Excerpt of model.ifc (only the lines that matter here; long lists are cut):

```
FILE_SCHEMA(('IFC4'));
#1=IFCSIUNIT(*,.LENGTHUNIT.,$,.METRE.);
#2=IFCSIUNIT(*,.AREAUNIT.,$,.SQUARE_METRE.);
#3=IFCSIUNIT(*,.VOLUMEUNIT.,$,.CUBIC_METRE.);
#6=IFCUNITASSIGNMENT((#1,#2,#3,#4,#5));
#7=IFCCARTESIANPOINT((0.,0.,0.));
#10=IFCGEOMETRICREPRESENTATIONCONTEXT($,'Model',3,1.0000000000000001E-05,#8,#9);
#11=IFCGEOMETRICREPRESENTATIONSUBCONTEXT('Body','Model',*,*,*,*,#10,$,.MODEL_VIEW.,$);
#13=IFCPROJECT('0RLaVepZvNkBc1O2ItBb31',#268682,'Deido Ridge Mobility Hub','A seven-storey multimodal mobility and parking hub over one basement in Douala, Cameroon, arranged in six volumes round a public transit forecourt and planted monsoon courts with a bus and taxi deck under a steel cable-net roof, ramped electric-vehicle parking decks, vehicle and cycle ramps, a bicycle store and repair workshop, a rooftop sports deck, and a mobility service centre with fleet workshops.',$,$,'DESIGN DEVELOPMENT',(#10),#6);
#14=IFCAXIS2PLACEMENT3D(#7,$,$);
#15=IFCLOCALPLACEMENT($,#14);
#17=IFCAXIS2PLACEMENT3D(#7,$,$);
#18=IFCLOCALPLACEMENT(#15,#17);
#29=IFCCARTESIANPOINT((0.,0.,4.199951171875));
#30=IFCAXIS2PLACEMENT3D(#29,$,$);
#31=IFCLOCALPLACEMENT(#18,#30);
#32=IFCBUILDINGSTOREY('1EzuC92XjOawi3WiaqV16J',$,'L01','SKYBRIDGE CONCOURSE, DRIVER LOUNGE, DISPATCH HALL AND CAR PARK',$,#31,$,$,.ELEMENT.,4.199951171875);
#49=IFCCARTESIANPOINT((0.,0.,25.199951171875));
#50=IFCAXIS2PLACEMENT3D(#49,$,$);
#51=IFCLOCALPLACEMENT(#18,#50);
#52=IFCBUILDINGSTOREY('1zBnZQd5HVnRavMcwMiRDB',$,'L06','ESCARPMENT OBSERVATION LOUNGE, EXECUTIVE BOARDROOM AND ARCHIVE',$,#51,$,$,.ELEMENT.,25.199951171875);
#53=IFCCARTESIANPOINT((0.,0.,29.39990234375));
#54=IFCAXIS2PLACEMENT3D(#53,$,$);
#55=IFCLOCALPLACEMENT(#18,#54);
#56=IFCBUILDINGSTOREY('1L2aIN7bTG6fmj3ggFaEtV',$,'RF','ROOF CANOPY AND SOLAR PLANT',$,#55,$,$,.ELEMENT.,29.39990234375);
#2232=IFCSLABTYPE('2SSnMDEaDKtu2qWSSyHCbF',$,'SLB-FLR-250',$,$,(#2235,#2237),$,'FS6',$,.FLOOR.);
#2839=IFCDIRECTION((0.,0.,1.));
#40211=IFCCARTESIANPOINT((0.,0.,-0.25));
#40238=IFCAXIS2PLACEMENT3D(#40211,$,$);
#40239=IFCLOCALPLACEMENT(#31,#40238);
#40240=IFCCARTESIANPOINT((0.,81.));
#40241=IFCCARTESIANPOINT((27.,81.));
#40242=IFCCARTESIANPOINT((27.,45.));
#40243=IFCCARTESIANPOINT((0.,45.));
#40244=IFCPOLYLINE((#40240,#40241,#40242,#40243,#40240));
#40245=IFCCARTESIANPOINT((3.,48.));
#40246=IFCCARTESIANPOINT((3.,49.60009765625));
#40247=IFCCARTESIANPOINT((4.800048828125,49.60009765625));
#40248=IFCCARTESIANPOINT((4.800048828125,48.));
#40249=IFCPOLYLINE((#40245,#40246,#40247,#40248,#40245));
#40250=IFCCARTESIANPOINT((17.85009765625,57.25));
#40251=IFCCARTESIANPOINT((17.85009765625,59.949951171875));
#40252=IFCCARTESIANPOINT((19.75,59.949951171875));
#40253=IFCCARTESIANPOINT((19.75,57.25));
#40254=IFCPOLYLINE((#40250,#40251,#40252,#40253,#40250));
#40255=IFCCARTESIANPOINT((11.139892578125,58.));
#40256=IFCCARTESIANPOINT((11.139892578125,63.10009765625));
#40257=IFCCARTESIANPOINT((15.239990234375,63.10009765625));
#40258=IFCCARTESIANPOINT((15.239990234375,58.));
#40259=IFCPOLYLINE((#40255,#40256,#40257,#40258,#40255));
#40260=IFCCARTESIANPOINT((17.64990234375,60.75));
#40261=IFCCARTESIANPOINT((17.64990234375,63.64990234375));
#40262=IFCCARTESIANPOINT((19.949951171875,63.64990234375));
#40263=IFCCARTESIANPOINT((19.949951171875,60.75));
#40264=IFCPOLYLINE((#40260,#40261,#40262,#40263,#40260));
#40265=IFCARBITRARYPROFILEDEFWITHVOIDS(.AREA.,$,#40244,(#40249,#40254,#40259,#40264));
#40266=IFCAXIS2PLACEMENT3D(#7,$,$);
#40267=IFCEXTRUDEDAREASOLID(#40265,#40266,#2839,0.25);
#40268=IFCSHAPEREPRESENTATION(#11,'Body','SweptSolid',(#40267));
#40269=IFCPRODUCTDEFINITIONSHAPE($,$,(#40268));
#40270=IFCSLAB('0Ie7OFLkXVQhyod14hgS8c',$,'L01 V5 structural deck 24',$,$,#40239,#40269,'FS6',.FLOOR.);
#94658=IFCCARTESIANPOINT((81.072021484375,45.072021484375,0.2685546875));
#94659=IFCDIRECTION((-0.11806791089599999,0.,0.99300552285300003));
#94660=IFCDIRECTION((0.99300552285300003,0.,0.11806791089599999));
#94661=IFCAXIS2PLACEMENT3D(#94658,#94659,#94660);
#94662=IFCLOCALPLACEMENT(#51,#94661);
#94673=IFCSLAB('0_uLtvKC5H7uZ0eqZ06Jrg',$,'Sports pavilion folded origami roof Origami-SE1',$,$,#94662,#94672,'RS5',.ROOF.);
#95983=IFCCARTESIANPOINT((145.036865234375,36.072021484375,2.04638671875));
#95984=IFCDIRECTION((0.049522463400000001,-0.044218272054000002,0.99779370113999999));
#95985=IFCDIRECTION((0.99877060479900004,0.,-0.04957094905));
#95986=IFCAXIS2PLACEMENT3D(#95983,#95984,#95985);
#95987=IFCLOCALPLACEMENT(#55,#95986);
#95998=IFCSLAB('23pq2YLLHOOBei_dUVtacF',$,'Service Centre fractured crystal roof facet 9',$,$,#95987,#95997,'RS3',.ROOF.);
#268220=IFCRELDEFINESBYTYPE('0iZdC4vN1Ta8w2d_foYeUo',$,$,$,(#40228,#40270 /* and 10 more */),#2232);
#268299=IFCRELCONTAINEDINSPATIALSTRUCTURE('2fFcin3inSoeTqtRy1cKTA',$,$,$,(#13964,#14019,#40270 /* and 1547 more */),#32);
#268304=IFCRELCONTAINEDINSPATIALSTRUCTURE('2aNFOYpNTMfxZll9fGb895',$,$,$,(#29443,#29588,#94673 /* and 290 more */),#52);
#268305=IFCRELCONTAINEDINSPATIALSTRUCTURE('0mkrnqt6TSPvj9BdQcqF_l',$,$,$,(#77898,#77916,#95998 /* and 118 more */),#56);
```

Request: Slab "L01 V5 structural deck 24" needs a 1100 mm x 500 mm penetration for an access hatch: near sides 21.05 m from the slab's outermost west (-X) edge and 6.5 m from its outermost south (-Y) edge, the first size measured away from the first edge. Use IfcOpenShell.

```python
import numpy as np
import ifcopenshell
import ifcopenshell.api.feature
import ifcopenshell.api.geometry
import ifcopenshell.api.root
import ifcopenshell.geom
import ifcopenshell.util.placement
import ifcopenshell.util.representation
import ifcopenshell.util.shape
import ifcopenshell.util.unit

model = ifcopenshell.open("model.ifc")
unit_scale = ifcopenshell.util.unit.calculate_unit_scale(model)
settings = ifcopenshell.geom.settings()


def volume(element):
    """Net volume in cubic metres, openings subtracted."""
    shape = ifcopenshell.geom.create_shape(settings, element)
    return ifcopenshell.util.shape.get_volume(shape.geometry)


slab = model.by_id(40270)
before = volume(slab)

# Extent in the slab's own axes, in metres. The edges named are its -X and -Y sides.
slab_shape = ifcopenshell.geom.create_shape(settings, slab)
vertices = ifcopenshell.util.shape.get_vertices(slab_shape.geometry)
x_min, y_min, bottom = vertices.min(axis=0)
top = vertices[:, 2].max()

opening = ifcopenshell.api.root.create_entity(model, ifc_class="IfcOpeningElement", name="Access hatch opening", predefined_type="OPENING")
context = ifcopenshell.util.representation.get_context(model, "Model", "Body", "MODEL_VIEW")
width, depth = 1.1, 0.5
outline = [(0.0, 0.0), (width, 0.0), (width, depth), (0.0, depth), (0.0, 0.0)]
# Overshoot both faces by 50 mm so the cut is clean.
shape = ifcopenshell.api.geometry.add_slab_representation(
    model, context=context, depth=top - bottom + 0.1, polyline=outline
)
ifcopenshell.api.geometry.assign_representation(model, product=opening, representation=shape)

matrix = ifcopenshell.util.placement.get_local_placement(slab.ObjectPlacement)
matrix[:, 3] = matrix @ np.append(np.array([x_min + 21.05, y_min + 6.5, bottom - 0.05]) / unit_scale, 1.0)
ifcopenshell.api.geometry.edit_object_placement(model, product=opening, matrix=matrix, is_si=False)
ifcopenshell.api.feature.add_feature(model, feature=opening, element=slab)

after = volume(slab)

print(f"slab volume {before:.3f} -> {after:.3f} m3")

model.write("model_v2.ifc")
```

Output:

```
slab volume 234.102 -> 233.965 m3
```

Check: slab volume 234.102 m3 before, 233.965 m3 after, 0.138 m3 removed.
